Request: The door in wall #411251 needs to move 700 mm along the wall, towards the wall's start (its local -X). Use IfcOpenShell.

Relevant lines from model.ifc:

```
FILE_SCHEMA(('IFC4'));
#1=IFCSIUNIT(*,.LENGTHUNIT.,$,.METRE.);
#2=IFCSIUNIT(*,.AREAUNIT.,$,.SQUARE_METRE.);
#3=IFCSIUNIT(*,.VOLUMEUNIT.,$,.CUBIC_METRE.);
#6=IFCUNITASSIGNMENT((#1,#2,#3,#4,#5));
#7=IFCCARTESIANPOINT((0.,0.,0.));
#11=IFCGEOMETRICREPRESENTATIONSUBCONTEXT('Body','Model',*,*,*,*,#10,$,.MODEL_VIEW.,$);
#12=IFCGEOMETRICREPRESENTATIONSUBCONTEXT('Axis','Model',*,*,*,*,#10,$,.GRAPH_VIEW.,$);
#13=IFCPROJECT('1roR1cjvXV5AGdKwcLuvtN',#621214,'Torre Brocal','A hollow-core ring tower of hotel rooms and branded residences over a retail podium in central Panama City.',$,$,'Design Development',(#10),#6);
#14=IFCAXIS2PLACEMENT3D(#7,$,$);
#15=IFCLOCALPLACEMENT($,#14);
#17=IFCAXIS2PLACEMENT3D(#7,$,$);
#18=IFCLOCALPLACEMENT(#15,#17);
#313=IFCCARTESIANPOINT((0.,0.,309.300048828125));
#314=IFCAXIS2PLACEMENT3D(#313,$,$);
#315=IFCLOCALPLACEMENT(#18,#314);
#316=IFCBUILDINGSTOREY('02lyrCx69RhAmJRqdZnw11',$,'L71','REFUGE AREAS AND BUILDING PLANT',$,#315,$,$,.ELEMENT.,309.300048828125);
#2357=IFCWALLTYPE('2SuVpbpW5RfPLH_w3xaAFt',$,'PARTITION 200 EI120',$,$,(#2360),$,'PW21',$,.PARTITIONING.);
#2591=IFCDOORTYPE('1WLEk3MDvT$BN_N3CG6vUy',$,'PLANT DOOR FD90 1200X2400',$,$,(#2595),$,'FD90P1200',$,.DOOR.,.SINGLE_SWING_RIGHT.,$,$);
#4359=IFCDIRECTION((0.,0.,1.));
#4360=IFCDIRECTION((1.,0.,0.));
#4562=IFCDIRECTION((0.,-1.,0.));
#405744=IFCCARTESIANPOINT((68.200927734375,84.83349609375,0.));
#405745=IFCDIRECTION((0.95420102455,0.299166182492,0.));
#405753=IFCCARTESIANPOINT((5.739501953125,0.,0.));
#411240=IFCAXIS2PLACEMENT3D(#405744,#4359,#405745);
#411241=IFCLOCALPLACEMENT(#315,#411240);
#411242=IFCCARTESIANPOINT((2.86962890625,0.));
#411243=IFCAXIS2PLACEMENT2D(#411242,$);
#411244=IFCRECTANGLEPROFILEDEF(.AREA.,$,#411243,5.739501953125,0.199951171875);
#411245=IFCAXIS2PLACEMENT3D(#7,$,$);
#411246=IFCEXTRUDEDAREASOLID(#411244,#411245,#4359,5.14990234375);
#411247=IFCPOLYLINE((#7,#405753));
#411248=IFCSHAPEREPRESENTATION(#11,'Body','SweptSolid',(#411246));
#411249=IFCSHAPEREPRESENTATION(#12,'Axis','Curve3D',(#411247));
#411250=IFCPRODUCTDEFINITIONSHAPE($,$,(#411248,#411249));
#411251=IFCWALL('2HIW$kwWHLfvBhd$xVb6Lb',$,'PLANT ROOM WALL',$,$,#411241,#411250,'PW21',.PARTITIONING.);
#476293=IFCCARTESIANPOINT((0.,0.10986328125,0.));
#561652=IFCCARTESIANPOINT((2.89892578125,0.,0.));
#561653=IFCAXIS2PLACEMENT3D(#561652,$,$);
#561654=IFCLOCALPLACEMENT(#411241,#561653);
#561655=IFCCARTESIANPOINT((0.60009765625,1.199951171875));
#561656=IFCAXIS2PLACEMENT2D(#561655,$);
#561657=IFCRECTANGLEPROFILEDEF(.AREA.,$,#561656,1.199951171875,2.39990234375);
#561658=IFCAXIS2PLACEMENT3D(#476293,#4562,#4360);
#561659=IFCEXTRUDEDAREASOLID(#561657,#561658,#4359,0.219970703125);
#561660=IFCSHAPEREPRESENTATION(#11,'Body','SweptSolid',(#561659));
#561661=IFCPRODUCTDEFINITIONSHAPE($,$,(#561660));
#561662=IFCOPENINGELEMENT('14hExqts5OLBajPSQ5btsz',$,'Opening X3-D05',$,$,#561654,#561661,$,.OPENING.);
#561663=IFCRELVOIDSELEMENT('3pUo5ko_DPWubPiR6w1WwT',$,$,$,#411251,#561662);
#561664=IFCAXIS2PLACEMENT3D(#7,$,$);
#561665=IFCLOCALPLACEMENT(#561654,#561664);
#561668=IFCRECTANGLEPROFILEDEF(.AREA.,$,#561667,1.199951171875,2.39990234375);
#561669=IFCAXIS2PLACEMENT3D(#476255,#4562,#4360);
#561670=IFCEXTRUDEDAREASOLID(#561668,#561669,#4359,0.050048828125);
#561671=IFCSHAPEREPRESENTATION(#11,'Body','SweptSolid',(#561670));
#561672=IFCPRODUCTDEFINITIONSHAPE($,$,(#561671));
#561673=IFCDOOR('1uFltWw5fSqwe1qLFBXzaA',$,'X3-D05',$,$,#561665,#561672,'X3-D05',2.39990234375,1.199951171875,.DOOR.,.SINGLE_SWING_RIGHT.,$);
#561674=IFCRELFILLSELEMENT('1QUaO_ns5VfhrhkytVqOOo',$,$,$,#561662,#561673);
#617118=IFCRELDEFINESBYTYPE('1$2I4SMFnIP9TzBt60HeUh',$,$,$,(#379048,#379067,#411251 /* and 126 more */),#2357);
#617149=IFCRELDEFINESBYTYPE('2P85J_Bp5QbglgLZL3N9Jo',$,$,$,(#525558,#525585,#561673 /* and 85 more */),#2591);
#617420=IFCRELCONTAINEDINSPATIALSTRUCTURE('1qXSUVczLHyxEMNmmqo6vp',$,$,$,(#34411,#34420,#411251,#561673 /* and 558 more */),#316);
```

```python
import ifcopenshell
import ifcopenshell.api.geometry
import ifcopenshell.util.placement
import ifcopenshell.util.unit

model = ifcopenshell.open("model.ifc")
unit_scale = ifcopenshell.util.unit.calculate_unit_scale(model)

door = model.by_guid("1uFltWw5fSqwe1qLFBXzaA")
opening = door.FillsVoids[0].RelatingOpeningElement
wall = opening.VoidsElements[0].RelatingBuildingElement

wall_matrix = ifcopenshell.util.placement.get_local_placement(wall.ObjectPlacement)
shift = wall_matrix[:3, 0] * -0.7 / unit_scale
before = ifcopenshell.util.placement.get_local_placement(door.ObjectPlacement)[:3, 3].copy()

# The door is placed relative to its opening, so it follows when the opening moves.
matrix = ifcopenshell.util.placement.get_local_placement(opening.ObjectPlacement)
matrix[:3, 3] += shift
ifcopenshell.api.geometry.edit_object_placement(
    model, product=opening, matrix=matrix, is_si=False, should_transform_children=True
)

after = ifcopenshell.util.placement.get_local_placement(door.ObjectPlacement)[:3, 3]
print("door moved by", (after - before).round(3) + 0.0)

model.write("model_rev.ifc")
```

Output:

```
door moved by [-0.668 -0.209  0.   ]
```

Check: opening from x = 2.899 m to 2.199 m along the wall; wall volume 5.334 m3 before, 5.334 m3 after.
